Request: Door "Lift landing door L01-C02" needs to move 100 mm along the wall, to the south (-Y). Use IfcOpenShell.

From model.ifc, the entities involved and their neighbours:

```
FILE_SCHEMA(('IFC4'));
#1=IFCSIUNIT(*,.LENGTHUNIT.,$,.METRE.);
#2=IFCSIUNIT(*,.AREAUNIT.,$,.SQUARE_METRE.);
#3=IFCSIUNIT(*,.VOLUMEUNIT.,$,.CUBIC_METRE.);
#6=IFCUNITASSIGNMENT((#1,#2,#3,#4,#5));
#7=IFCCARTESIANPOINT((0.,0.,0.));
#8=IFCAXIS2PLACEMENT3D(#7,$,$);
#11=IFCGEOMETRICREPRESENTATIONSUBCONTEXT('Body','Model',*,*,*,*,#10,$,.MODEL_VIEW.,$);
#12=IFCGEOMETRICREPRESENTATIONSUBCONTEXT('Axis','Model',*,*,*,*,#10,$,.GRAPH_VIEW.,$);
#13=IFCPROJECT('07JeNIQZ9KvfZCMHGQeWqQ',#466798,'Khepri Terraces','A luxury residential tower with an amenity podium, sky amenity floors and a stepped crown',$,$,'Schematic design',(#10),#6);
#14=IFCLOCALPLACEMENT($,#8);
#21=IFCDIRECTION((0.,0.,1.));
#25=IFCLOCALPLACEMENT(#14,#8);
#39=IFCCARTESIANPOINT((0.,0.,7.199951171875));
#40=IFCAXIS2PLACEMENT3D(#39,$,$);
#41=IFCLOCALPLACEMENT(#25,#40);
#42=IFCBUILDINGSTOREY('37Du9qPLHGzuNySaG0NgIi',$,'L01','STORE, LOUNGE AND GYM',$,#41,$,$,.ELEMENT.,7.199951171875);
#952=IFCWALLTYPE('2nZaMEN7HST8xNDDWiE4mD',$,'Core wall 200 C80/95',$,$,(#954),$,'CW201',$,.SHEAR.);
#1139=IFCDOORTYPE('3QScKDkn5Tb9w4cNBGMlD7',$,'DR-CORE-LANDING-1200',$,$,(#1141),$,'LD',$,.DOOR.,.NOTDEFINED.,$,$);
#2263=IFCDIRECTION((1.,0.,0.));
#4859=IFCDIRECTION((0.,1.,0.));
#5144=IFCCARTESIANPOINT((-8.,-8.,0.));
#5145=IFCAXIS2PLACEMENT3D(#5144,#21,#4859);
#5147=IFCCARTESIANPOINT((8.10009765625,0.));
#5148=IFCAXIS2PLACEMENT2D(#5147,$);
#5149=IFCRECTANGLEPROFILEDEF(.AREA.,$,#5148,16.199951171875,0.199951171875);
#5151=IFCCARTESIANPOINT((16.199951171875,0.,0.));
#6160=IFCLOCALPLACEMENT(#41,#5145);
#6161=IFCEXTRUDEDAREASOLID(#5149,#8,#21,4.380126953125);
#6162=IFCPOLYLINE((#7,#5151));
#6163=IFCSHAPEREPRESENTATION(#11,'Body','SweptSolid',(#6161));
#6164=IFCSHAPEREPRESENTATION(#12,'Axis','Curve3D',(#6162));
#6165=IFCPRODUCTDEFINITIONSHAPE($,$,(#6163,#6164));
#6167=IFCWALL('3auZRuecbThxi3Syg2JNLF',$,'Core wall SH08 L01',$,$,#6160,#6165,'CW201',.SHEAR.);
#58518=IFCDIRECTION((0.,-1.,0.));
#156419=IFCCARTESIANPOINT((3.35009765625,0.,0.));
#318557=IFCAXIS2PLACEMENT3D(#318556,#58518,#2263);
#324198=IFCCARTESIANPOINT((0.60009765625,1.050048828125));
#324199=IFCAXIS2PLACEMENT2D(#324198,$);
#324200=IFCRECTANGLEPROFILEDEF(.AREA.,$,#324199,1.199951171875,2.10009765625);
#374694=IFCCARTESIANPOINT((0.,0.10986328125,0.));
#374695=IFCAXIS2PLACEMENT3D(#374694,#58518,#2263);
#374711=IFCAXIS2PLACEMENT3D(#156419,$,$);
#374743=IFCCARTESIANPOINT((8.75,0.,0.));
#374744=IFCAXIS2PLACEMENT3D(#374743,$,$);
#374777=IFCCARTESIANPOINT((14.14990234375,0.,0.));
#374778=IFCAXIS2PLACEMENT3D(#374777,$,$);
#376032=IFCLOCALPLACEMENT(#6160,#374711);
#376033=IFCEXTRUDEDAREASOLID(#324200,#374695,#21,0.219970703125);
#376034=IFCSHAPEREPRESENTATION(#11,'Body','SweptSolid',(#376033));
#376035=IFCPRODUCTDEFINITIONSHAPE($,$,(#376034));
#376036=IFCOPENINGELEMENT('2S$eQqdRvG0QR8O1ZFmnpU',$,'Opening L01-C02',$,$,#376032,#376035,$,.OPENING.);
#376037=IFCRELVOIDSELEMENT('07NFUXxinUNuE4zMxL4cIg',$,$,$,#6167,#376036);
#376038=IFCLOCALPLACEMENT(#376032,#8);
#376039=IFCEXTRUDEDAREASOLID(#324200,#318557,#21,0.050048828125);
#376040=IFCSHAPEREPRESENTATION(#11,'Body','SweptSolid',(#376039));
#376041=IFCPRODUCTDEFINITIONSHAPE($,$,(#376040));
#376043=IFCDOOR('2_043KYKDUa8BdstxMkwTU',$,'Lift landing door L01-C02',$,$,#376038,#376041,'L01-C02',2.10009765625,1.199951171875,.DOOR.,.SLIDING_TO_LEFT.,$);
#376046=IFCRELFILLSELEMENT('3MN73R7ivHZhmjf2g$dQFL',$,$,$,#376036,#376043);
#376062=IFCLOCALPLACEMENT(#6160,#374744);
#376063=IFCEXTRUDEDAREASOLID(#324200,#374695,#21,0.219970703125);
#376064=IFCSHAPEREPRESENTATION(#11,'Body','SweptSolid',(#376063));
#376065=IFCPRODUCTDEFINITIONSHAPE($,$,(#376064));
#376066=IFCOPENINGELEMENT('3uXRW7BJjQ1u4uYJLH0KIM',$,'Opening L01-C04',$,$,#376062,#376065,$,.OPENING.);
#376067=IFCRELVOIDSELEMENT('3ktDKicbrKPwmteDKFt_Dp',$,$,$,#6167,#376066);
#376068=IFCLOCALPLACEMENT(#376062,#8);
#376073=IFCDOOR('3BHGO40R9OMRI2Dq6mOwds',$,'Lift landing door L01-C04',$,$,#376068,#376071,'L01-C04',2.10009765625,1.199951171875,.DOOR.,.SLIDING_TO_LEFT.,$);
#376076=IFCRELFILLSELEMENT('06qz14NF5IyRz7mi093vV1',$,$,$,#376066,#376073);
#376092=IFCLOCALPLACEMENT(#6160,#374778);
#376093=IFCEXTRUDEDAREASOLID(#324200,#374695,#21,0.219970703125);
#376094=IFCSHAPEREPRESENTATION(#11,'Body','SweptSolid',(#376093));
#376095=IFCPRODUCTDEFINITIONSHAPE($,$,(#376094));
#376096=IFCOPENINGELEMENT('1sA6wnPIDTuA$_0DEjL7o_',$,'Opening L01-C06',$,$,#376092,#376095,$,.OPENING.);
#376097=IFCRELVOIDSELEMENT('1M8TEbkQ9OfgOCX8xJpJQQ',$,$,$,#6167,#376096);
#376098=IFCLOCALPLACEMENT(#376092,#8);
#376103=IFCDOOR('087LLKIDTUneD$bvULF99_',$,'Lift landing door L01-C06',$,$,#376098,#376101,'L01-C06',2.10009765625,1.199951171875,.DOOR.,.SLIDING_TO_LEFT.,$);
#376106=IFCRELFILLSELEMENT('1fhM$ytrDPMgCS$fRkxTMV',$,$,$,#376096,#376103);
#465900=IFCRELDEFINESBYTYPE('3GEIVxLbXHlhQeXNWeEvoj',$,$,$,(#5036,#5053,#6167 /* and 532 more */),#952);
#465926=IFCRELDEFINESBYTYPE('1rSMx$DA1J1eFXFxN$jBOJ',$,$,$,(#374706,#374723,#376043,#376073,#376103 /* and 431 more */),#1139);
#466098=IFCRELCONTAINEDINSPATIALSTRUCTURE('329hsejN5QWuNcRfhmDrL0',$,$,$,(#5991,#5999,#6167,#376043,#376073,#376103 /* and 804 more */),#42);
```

```python
import ifcopenshell
import ifcopenshell.api.geometry
import ifcopenshell.util.placement
import ifcopenshell.util.unit

model = ifcopenshell.open("model.ifc")
unit_scale = ifcopenshell.util.unit.calculate_unit_scale(model)

door = model.by_guid("2_043KYKDUa8BdstxMkwTU")
opening = door.FillsVoids[0].RelatingOpeningElement
wall = opening.VoidsElements[0].RelatingBuildingElement

wall_matrix = ifcopenshell.util.placement.get_local_placement(wall.ObjectPlacement)
shift = wall_matrix[:3, 0] * -0.1 / unit_scale
before = ifcopenshell.util.placement.get_local_placement(door.ObjectPlacement)[:3, 3].copy()

# The door is placed relative to its opening, so it follows when the opening moves.
matrix = ifcopenshell.util.placement.get_local_placement(opening.ObjectPlacement)
matrix[:3, 3] += shift
ifcopenshell.api.geometry.edit_object_placement(
    model, product=opening, matrix=matrix, is_si=False, should_transform_children=True
)

after = ifcopenshell.util.placement.get_local_placement(door.ObjectPlacement)[:3, 3]
print("door moved by", (after - before).round(3) + 0.0)

model.write("model_v2.ifc")
```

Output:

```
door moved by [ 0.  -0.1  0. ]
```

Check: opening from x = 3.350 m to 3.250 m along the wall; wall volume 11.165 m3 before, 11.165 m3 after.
